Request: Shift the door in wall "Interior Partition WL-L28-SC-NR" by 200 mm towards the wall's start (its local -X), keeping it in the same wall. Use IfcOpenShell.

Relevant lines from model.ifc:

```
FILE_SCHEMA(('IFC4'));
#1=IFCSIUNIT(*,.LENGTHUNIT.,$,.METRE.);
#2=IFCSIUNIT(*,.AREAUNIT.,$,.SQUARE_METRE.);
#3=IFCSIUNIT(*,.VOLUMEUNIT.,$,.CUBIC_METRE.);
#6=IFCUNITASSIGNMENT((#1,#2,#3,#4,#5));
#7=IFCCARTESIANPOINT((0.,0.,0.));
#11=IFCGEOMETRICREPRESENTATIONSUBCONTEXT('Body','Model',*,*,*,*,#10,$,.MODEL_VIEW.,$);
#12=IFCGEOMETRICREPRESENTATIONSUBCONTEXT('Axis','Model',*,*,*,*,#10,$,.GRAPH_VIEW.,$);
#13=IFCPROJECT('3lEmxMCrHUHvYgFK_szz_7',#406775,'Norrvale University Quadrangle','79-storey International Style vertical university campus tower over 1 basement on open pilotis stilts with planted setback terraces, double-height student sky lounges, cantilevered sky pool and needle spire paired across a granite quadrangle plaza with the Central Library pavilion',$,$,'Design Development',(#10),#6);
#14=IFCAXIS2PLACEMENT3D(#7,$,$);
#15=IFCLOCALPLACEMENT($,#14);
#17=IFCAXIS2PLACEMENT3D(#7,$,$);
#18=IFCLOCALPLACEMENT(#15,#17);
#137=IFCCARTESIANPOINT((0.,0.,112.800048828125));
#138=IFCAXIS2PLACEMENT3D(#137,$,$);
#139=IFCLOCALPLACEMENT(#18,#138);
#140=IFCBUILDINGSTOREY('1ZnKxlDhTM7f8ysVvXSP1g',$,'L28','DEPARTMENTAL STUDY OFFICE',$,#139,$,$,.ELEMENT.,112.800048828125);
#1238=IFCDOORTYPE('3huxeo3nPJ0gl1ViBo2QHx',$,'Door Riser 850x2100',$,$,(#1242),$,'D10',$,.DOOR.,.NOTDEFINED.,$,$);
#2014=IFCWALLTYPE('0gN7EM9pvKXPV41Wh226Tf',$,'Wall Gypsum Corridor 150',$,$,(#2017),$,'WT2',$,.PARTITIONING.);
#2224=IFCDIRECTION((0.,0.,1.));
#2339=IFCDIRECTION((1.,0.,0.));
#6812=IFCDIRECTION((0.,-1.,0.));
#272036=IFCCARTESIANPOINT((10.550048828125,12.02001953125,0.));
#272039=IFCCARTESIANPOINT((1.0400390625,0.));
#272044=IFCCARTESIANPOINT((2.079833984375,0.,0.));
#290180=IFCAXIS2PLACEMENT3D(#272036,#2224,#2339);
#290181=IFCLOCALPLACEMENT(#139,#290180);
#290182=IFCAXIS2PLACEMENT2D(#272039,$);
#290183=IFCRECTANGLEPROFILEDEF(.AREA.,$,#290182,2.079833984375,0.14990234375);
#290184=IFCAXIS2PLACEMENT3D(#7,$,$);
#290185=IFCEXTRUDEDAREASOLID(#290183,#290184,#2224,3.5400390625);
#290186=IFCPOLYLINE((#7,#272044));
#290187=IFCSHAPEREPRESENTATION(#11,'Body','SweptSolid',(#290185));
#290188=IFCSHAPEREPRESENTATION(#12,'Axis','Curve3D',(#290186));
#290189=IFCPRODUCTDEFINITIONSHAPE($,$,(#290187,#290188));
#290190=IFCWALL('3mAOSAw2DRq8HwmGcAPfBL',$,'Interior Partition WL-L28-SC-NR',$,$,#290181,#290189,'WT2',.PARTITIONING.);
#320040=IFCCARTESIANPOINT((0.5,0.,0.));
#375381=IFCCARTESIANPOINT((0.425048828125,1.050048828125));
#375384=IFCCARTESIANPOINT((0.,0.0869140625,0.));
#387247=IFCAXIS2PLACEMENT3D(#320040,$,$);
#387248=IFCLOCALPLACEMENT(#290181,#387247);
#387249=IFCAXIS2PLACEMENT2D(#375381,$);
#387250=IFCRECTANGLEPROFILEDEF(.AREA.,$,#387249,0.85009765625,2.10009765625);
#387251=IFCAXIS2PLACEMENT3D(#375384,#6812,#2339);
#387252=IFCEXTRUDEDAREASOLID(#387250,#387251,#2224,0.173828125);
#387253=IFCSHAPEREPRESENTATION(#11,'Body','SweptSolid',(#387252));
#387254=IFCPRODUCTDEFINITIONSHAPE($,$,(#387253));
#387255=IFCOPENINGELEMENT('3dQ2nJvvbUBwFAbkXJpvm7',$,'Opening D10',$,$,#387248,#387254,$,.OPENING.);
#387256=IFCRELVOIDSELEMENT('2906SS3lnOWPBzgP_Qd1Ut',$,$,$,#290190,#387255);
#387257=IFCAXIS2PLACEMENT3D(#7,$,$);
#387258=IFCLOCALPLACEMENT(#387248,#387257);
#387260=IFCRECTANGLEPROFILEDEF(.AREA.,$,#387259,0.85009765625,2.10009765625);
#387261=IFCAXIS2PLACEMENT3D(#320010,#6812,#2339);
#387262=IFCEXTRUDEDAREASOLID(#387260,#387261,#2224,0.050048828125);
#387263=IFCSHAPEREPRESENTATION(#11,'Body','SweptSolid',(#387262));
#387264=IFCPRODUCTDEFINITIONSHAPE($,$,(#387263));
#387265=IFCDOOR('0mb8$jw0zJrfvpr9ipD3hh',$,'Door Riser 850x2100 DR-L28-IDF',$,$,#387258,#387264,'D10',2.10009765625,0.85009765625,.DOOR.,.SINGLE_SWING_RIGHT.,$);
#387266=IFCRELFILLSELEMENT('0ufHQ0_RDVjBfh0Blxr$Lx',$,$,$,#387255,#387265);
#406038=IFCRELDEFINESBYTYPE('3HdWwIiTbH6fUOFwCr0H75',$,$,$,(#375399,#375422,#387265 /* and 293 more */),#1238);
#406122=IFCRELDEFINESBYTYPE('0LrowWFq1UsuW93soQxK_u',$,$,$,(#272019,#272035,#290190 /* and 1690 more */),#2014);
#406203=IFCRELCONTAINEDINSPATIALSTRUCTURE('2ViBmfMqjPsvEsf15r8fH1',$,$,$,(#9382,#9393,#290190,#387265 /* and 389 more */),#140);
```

```python
import ifcopenshell
import ifcopenshell.api.geometry
import ifcopenshell.util.placement
import ifcopenshell.util.unit

model = ifcopenshell.open("model.ifc")
unit_scale = ifcopenshell.util.unit.calculate_unit_scale(model)

door = model.by_id(387265)
opening = door.FillsVoids[0].RelatingOpeningElement
wall = opening.VoidsElements[0].RelatingBuildingElement

wall_matrix = ifcopenshell.util.placement.get_local_placement(wall.ObjectPlacement)
shift = wall_matrix[:3, 0] * -0.2 / unit_scale
before = ifcopenshell.util.placement.get_local_placement(door.ObjectPlacement)[:3, 3].copy()

# The door is placed relative to its opening, so it follows when the opening moves.
matrix = ifcopenshell.util.placement.get_local_placement(opening.ObjectPlacement)
matrix[:3, 3] += shift
ifcopenshell.api.geometry.edit_object_placement(
    model, product=opening, matrix=matrix, is_si=False, should_transform_children=True
)

after = ifcopenshell.util.placement.get_local_placement(door.ObjectPlacement)[:3, 3]
print("door moved by", (after - before).round(3) + 0.0)

model.write("model_v2.ifc")
```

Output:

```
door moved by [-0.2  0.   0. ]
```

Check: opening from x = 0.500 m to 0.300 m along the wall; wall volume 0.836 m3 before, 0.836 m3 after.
